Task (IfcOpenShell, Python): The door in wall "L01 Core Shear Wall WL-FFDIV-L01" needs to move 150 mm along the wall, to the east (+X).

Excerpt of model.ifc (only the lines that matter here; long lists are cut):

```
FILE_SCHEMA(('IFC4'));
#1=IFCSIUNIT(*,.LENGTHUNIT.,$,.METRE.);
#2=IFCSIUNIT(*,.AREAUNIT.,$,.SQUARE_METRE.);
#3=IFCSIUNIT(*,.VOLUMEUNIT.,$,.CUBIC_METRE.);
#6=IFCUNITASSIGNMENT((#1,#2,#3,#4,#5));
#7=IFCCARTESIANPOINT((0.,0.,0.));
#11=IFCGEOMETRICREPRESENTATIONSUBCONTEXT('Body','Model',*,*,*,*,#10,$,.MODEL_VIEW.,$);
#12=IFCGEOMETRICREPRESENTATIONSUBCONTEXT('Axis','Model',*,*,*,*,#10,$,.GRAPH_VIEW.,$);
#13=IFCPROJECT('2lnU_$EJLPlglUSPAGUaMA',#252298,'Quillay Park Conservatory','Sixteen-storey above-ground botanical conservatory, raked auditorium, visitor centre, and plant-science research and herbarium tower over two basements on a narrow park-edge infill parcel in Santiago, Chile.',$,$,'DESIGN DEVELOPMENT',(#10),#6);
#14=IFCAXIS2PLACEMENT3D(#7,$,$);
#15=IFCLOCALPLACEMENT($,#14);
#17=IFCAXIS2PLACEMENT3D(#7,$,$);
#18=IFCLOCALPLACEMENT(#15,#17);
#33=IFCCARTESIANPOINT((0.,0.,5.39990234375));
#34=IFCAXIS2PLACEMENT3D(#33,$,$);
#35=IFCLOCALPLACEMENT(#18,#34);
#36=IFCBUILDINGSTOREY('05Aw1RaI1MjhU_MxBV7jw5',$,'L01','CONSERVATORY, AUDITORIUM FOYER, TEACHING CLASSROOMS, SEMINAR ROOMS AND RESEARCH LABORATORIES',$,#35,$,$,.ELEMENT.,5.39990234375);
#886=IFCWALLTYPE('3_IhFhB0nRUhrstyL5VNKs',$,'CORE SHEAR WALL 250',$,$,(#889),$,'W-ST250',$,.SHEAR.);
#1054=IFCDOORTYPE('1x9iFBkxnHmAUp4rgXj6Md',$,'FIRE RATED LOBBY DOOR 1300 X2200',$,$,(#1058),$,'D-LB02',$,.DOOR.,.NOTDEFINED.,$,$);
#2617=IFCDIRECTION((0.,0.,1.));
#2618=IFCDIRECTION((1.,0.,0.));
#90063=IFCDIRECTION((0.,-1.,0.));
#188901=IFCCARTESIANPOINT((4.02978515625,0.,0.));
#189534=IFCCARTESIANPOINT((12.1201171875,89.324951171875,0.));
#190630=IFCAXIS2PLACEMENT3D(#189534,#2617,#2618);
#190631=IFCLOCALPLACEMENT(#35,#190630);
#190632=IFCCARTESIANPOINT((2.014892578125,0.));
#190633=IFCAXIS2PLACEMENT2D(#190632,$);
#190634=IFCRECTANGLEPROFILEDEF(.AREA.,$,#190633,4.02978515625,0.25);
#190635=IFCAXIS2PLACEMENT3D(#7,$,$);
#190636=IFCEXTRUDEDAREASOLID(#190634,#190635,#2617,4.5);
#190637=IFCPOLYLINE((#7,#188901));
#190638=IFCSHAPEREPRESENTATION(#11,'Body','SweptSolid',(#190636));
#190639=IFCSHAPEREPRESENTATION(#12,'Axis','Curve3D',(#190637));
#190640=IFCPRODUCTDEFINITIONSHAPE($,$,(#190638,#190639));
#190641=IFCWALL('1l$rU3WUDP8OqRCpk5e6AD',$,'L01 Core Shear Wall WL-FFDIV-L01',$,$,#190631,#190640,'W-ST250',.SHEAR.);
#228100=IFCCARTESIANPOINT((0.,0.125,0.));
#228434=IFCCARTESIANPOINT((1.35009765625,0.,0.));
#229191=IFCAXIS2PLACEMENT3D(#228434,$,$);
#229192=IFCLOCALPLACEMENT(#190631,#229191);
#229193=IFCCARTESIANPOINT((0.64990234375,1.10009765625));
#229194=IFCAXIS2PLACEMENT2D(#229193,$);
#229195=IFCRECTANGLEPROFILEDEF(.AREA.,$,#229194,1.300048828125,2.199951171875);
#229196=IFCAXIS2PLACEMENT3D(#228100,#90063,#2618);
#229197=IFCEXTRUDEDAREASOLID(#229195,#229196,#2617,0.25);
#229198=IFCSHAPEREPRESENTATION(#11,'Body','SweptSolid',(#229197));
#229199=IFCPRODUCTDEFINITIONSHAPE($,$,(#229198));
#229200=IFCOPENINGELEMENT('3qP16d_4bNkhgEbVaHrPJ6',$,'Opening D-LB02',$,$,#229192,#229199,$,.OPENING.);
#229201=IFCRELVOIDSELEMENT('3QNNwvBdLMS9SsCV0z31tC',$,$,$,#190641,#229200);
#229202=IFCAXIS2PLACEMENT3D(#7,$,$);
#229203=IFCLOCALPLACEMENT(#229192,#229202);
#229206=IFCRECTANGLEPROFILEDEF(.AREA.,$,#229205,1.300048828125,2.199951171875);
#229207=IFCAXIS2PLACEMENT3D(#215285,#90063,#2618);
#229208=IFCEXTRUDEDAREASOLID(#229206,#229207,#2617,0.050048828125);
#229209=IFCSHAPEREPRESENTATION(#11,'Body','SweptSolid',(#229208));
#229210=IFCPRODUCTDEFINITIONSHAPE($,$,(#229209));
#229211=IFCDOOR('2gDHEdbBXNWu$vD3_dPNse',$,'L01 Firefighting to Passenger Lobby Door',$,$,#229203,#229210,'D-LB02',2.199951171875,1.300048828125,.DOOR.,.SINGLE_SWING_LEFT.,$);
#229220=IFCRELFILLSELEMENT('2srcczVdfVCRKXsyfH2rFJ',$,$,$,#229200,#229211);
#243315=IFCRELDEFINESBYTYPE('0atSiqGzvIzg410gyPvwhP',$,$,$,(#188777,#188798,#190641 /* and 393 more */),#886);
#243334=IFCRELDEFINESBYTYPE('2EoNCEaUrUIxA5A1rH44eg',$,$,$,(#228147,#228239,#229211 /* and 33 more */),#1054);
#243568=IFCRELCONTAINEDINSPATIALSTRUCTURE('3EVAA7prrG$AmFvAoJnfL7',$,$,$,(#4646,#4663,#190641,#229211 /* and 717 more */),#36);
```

```python
import ifcopenshell
import ifcopenshell.api.geometry
import ifcopenshell.util.placement
import ifcopenshell.util.unit

model = ifcopenshell.open("model.ifc")
unit_scale = ifcopenshell.util.unit.calculate_unit_scale(model)

door = model.by_id(229211)
opening = door.FillsVoids[0].RelatingOpeningElement
wall = opening.VoidsElements[0].RelatingBuildingElement

wall_matrix = ifcopenshell.util.placement.get_local_placement(wall.ObjectPlacement)
shift = wall_matrix[:3, 0] * 0.15 / unit_scale
before = ifcopenshell.util.placement.get_local_placement(door.ObjectPlacement)[:3, 3].copy()

# The door is placed relative to its opening, so it follows when the opening moves.
matrix = ifcopenshell.util.placement.get_local_placement(opening.ObjectPlacement)
matrix[:3, 3] += shift
ifcopenshell.api.geometry.edit_object_placement(
    model, product=opening, matrix=matrix, is_si=False, should_transform_children=True
)

after = ifcopenshell.util.placement.get_local_placement(door.ObjectPlacement)[:3, 3]
print("door moved by", (after - before).round(3) + 0.0)

model.write("model_v2.ifc")
```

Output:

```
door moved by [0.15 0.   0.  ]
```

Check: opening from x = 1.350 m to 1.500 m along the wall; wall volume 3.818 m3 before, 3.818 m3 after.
